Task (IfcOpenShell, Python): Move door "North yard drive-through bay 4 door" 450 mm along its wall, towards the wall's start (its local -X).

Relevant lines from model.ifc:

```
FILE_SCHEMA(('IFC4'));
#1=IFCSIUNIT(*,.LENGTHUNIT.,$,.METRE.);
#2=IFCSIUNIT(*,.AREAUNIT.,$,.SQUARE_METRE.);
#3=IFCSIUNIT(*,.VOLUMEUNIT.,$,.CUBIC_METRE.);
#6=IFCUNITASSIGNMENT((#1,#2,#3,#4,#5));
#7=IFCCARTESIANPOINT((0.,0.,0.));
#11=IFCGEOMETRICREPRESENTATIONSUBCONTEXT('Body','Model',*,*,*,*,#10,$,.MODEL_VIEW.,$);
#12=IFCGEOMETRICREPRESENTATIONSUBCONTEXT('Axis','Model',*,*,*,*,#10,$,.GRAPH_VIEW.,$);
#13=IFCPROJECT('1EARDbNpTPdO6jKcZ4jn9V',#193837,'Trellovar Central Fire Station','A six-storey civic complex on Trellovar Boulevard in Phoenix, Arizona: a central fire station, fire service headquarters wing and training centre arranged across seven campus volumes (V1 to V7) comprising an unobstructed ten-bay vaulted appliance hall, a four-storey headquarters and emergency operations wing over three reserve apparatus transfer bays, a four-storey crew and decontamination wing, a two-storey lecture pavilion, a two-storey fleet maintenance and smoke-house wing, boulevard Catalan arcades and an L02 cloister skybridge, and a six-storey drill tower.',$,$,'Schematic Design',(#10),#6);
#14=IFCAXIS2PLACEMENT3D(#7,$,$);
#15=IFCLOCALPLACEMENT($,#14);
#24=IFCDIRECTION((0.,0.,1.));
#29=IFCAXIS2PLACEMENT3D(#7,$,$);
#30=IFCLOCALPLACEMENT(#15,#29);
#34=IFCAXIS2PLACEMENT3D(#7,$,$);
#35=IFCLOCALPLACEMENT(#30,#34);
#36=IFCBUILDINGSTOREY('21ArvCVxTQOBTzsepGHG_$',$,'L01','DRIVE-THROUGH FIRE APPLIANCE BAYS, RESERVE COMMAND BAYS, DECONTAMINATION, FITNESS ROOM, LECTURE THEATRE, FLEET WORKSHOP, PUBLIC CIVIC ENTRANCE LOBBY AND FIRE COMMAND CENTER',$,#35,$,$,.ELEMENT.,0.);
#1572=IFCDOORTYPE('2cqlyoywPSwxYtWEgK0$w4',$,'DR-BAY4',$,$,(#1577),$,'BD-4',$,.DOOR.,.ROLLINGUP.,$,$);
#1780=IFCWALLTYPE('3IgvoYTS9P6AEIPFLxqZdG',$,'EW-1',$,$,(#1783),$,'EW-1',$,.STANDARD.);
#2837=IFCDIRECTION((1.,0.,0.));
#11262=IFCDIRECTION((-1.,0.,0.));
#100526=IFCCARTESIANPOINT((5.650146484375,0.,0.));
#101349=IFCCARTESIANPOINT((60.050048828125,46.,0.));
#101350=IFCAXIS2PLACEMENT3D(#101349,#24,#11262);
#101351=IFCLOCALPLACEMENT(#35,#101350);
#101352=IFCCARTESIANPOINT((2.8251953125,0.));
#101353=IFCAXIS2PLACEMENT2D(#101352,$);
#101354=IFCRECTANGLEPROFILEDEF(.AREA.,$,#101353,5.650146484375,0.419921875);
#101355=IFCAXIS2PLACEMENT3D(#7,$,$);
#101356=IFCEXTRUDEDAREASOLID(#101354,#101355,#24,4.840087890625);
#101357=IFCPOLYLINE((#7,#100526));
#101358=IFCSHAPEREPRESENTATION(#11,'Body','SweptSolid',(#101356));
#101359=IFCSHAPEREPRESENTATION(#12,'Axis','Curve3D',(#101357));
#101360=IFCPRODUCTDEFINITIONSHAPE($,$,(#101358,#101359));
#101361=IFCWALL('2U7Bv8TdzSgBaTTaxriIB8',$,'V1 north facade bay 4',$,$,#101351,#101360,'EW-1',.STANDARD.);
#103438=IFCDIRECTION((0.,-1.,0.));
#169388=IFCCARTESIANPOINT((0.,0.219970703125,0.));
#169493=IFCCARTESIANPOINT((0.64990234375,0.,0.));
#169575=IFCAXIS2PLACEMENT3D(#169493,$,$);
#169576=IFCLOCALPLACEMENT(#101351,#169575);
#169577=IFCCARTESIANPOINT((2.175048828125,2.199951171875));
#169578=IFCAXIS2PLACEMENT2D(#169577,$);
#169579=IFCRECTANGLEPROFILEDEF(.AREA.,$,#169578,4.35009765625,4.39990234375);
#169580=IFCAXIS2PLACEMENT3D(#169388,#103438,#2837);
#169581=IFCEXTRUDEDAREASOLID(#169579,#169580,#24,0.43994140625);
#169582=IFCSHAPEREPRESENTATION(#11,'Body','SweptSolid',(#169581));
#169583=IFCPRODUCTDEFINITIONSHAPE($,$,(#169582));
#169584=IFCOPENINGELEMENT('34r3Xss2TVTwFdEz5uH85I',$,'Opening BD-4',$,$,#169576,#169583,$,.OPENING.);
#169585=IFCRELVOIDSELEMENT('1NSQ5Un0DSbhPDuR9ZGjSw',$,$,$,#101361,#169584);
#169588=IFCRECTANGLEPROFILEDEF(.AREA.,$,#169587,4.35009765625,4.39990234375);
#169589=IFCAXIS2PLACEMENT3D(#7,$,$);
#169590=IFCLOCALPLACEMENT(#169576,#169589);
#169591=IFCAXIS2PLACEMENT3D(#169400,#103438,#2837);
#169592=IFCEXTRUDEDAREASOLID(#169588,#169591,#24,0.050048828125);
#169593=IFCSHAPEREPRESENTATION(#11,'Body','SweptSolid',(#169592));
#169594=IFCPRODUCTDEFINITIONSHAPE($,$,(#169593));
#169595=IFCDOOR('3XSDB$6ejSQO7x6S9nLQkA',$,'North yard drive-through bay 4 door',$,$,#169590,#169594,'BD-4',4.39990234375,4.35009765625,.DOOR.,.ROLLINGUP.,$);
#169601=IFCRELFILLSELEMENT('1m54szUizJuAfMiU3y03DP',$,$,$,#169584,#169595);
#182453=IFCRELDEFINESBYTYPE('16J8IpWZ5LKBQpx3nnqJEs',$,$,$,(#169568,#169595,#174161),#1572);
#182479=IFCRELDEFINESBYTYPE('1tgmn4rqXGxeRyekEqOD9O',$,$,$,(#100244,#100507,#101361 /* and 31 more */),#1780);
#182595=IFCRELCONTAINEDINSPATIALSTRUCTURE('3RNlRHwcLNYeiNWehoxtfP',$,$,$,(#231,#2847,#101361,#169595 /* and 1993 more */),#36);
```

```python
import ifcopenshell
import ifcopenshell.api.geometry
import ifcopenshell.util.placement
import ifcopenshell.util.unit

model = ifcopenshell.open("model.ifc")
unit_scale = ifcopenshell.util.unit.calculate_unit_scale(model)

door = model.by_guid("3XSDB$6ejSQO7x6S9nLQkA")
opening = door.FillsVoids[0].RelatingOpeningElement
wall = opening.VoidsElements[0].RelatingBuildingElement

wall_matrix = ifcopenshell.util.placement.get_local_placement(wall.ObjectPlacement)
shift = wall_matrix[:3, 0] * -0.45 / unit_scale
before = ifcopenshell.util.placement.get_local_placement(door.ObjectPlacement)[:3, 3].copy()

# The door is placed relative to its opening, so it follows when the opening moves.
matrix = ifcopenshell.util.placement.get_local_placement(opening.ObjectPlacement)
matrix[:3, 3] += shift
ifcopenshell.api.geometry.edit_object_placement(
    model, product=opening, matrix=matrix, is_si=False, should_transform_children=True
)

after = ifcopenshell.util.placement.get_local_placement(door.ObjectPlacement)[:3, 3]
print("door moved by", (after - before).round(3) + 0.0)

model.write("model_edited.ifc")
```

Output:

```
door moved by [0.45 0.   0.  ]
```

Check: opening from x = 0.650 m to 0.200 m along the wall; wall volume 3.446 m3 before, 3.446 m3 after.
